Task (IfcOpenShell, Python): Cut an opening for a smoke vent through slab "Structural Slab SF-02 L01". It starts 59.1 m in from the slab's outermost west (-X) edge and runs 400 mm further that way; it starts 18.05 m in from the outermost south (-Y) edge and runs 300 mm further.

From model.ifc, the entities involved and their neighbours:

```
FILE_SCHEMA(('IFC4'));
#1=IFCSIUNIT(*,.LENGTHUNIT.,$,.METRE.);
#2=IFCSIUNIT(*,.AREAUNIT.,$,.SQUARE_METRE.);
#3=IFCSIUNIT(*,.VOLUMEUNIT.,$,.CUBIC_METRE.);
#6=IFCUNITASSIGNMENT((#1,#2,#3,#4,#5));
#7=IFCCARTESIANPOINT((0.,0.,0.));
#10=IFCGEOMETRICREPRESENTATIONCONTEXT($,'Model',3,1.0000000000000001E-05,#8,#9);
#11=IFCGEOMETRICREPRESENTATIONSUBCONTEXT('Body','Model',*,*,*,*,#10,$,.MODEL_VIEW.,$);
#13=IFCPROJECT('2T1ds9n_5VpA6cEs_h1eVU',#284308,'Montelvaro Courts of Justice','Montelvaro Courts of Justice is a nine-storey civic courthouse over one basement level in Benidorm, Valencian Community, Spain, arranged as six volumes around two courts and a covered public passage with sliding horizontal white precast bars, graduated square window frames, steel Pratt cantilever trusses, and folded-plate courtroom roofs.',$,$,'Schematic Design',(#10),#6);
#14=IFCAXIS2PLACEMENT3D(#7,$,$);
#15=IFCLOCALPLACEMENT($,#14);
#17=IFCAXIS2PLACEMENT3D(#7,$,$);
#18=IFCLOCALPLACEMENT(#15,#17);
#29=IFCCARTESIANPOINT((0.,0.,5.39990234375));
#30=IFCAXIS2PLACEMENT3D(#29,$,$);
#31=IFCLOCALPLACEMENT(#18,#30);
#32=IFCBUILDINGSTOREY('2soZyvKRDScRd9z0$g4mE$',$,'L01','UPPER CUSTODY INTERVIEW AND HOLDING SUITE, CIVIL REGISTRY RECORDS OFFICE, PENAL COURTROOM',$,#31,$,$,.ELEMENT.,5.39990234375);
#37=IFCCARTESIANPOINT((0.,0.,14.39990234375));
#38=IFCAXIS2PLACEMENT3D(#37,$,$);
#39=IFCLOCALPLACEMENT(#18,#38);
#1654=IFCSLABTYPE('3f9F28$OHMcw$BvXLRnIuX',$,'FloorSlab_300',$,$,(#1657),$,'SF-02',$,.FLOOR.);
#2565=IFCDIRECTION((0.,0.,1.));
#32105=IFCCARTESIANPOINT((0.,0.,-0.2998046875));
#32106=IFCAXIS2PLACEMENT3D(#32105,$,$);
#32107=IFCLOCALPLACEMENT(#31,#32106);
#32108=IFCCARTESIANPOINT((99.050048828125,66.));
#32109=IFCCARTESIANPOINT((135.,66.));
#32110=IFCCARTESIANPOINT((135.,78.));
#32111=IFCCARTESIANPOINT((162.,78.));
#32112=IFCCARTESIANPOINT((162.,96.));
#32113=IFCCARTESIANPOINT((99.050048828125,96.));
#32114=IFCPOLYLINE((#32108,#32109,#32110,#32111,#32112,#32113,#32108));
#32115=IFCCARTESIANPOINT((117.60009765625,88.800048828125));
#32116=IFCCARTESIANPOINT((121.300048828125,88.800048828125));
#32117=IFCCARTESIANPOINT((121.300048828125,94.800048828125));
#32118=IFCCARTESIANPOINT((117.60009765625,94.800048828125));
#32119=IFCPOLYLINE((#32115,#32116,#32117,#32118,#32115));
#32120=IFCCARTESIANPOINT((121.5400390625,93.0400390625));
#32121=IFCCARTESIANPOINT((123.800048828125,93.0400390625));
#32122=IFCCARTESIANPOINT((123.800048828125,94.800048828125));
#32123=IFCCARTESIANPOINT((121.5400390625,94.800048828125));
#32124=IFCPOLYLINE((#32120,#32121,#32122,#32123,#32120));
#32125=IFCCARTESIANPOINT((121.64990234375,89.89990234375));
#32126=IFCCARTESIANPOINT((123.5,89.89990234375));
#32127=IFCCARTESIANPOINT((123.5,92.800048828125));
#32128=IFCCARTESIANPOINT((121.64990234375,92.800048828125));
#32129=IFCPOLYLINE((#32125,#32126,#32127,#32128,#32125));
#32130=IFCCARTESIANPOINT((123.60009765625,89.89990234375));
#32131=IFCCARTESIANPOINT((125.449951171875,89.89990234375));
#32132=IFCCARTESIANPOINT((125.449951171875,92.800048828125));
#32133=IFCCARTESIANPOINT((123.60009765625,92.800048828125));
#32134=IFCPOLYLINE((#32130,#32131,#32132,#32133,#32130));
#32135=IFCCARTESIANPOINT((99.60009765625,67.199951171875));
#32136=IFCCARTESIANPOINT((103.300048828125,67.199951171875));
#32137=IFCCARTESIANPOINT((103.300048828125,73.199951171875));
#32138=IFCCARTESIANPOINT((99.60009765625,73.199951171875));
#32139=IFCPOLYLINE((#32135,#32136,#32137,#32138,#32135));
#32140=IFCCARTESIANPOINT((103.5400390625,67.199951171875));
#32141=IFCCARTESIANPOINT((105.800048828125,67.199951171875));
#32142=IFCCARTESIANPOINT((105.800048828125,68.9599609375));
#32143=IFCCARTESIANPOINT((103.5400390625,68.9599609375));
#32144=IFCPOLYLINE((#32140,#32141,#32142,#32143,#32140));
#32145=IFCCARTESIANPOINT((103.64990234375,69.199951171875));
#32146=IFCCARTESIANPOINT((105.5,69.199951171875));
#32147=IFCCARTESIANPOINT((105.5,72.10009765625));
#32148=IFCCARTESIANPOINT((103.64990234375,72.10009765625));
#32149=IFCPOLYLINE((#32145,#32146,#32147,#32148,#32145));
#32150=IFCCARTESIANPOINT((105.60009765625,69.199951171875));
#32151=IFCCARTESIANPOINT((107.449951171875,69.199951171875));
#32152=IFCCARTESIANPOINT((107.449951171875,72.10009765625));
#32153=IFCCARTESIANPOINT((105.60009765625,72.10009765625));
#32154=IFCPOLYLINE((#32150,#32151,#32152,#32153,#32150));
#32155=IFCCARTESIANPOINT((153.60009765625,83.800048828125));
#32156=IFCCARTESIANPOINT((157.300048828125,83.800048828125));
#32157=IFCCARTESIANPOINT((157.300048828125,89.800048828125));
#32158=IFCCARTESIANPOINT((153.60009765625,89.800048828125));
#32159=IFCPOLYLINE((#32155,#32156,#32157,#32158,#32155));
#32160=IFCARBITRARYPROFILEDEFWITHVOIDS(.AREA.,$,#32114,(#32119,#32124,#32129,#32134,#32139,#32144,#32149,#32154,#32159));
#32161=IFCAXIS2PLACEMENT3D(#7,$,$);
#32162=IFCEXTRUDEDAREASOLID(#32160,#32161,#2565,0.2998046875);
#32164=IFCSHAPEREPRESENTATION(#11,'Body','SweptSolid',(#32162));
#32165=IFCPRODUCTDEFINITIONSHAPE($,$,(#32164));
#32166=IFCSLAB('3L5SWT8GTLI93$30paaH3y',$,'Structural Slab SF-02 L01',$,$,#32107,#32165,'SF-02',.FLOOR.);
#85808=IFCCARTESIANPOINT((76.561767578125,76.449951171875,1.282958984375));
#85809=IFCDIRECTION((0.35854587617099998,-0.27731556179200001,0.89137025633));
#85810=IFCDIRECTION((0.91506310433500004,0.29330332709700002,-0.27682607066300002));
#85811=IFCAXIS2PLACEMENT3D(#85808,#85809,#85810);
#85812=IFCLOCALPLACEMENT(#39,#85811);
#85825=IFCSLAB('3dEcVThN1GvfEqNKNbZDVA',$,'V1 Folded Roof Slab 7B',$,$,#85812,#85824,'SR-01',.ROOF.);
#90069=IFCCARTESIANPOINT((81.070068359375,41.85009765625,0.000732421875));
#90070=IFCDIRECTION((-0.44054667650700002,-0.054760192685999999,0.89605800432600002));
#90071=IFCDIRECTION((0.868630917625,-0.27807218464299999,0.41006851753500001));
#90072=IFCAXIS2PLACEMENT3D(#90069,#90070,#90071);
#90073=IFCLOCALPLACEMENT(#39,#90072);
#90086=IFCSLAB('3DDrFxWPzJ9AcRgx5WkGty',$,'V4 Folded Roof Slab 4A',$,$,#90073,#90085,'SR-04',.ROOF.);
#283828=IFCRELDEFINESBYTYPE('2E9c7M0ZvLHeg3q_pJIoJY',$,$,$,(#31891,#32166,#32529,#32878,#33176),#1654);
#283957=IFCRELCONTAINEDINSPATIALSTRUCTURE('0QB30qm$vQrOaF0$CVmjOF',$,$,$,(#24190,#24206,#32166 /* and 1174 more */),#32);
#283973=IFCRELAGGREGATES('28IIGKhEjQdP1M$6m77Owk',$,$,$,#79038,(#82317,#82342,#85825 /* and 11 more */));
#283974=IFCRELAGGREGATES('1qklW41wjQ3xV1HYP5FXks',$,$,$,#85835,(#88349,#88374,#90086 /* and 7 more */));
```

```python
import numpy as np
import ifcopenshell
import ifcopenshell.api.feature
import ifcopenshell.api.geometry
import ifcopenshell.api.root
import ifcopenshell.geom
import ifcopenshell.util.placement
import ifcopenshell.util.representation
import ifcopenshell.util.shape
import ifcopenshell.util.unit

model = ifcopenshell.open("model.ifc")
unit_scale = ifcopenshell.util.unit.calculate_unit_scale(model)
settings = ifcopenshell.geom.settings()


def volume(element):
    """Net volume in cubic metres, openings subtracted."""
    shape = ifcopenshell.geom.create_shape(settings, element)
    return ifcopenshell.util.shape.get_volume(shape.geometry)


slab = model.by_guid("3L5SWT8GTLI93$30paaH3y")
before = volume(slab)

# Extent in the slab's own axes, in metres. The edges named are its -X and -Y sides.
slab_shape = ifcopenshell.geom.create_shape(settings, slab)
vertices = ifcopenshell.util.shape.get_vertices(slab_shape.geometry)
x_min, y_min, bottom = vertices.min(axis=0)
top = vertices[:, 2].max()

opening = ifcopenshell.api.root.create_entity(model, ifc_class="IfcOpeningElement", name="Smoke vent opening", predefined_type="OPENING")
context = ifcopenshell.util.representation.get_context(model, "Model", "Body", "MODEL_VIEW")
width, depth = 0.4, 0.3
outline = [(0.0, 0.0), (width, 0.0), (width, depth), (0.0, depth), (0.0, 0.0)]
# Overshoot both faces by 50 mm so the cut is clean.
shape = ifcopenshell.api.geometry.add_slab_representation(
    model, context=context, depth=top - bottom + 0.1, polyline=outline
)
ifcopenshell.api.geometry.assign_representation(model, product=opening, representation=shape)

matrix = ifcopenshell.util.placement.get_local_placement(slab.ObjectPlacement)
matrix[:, 3] = matrix @ np.append(np.array([x_min + 59.1, y_min + 18.05, bottom - 0.05]) / unit_scale, 1.0)
ifcopenshell.api.geometry.edit_object_placement(model, product=opening, matrix=matrix, is_si=False)
ifcopenshell.api.feature.add_feature(model, feature=opening, element=slab)

after = volume(slab)

print(f"slab volume {before:.3f} -> {after:.3f} m3")

model.write("model_rev.ifc")
```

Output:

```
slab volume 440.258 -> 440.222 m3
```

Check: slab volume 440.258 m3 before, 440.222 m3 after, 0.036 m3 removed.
